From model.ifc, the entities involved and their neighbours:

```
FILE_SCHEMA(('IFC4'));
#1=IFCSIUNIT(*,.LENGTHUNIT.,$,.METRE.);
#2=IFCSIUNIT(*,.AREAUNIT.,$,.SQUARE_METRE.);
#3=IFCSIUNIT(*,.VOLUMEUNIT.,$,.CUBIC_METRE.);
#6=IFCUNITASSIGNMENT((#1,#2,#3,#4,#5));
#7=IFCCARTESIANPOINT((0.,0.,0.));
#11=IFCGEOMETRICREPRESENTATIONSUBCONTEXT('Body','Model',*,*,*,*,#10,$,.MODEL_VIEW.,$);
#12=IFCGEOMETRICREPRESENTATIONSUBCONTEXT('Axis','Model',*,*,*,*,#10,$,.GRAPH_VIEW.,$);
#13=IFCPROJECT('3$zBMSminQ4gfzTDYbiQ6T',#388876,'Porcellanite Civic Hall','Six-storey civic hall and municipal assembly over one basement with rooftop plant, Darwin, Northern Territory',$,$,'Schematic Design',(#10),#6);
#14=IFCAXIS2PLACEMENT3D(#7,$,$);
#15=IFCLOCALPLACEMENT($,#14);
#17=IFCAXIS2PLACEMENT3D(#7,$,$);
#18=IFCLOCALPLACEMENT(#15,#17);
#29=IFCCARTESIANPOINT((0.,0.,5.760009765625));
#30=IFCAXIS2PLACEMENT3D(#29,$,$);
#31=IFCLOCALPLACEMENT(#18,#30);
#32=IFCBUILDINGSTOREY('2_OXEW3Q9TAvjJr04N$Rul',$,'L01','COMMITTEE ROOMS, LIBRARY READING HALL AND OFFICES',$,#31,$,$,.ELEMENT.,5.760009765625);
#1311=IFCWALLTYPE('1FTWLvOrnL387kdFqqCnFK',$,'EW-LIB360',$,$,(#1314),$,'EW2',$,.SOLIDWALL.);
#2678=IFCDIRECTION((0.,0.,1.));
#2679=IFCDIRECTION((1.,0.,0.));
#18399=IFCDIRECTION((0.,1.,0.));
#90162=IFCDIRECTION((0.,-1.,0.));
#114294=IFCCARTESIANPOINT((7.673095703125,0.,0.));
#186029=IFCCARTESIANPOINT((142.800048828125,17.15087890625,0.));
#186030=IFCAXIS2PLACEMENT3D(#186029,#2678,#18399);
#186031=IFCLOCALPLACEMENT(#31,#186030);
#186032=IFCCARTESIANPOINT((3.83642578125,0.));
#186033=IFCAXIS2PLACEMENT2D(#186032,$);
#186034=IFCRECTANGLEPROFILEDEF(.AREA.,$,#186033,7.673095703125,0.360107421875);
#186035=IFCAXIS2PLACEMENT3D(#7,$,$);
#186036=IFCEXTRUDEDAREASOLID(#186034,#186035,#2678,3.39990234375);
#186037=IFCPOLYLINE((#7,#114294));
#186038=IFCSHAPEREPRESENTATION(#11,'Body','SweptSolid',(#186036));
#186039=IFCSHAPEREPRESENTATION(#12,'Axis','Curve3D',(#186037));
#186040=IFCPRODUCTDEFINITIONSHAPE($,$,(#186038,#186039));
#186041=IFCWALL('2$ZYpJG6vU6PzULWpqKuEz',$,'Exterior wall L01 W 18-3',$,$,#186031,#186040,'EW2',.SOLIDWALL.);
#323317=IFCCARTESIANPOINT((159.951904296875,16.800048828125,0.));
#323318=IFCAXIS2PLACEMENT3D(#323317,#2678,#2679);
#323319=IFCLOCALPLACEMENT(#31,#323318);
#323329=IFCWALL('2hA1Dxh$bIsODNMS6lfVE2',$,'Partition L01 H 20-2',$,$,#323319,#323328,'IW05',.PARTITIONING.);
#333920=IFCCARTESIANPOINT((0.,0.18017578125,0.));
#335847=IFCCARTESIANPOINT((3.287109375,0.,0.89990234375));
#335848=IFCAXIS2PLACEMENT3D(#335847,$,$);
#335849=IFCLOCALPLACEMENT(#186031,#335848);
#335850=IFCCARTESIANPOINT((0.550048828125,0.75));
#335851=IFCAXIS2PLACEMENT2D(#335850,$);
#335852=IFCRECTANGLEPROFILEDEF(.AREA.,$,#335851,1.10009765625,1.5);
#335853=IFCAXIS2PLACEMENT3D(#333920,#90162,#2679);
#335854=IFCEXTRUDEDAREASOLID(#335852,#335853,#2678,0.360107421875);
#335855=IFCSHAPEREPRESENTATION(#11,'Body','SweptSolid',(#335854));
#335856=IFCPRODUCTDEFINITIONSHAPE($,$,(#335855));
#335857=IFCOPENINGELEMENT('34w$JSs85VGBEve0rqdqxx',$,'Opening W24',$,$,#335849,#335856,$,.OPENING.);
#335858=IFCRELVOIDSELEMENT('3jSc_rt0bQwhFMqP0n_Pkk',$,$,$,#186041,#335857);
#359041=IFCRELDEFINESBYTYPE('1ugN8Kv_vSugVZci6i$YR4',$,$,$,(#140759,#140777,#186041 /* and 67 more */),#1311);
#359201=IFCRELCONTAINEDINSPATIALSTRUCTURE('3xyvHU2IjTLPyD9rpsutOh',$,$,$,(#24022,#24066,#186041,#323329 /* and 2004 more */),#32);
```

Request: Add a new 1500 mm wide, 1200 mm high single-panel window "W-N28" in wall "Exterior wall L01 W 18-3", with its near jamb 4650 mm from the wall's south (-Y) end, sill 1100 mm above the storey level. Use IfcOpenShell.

```python
import numpy as np
import ifcopenshell
import ifcopenshell.api.feature
import ifcopenshell.api.geometry
import ifcopenshell.api.root
import ifcopenshell.api.spatial
import ifcopenshell.geom
import ifcopenshell.util.element
import ifcopenshell.util.placement
import ifcopenshell.util.representation
import ifcopenshell.util.shape
import ifcopenshell.util.unit

model = ifcopenshell.open("model.ifc")
unit_scale = ifcopenshell.util.unit.calculate_unit_scale(model)
settings = ifcopenshell.geom.settings()


def volume(element):
    """Net volume in cubic metres, openings subtracted."""
    shape = ifcopenshell.geom.create_shape(settings, element)
    return ifcopenshell.util.shape.get_volume(shape.geometry)


wall = model.by_guid("2$ZYpJG6vU6PzULWpqKuEz")
storey = ifcopenshell.util.element.get_container(wall, ifc_class="IfcBuildingStorey")
context = ifcopenshell.util.representation.get_context(model, "Model", "Body", "MODEL_VIEW")
before = volume(wall)

width, height, from_end, sill = 1.5, 1.2, 4.65, 1.1  # metres

# The wall runs along its own X axis, and the end named is its -X end.
wall_shape = ifcopenshell.geom.create_shape(settings, wall)
x, y, z = ifcopenshell.util.shape.get_vertices(wall_shape.geometry).T
start = x.min() + from_end
face, thickness = float(y.min()), float(y.max() - y.min())
wall_matrix = ifcopenshell.util.placement.get_local_placement(wall.ObjectPlacement)
level = ifcopenshell.util.placement.get_local_placement(storey.ObjectPlacement)[2, 3]


def in_wall(x, y):
    """Placement at x, y metres in the wall's axes, at sill height."""
    matrix = wall_matrix.copy()
    matrix[:, 3] = wall_matrix @ np.array([x / unit_scale, y / unit_scale, 0.0, 1.0])
    matrix[2, 3] = level + sill / unit_scale
    return matrix


# Opening: a box that overshoots both wall faces by 50 mm.
opening = ifcopenshell.api.root.create_entity(model, ifc_class="IfcOpeningElement", predefined_type="OPENING")
box = ifcopenshell.api.geometry.add_wall_representation(
    model, context=context, length=width, height=height, thickness=thickness + 0.1
)
ifcopenshell.api.geometry.assign_representation(model, product=opening, representation=box)
ifcopenshell.api.geometry.edit_object_placement(model, product=opening, matrix=in_wall(start, face - 0.05), is_si=False)
ifcopenshell.api.feature.add_feature(model, feature=opening, element=wall)

window = ifcopenshell.api.root.create_entity(model, ifc_class="IfcWindow", name="W-N28", predefined_type="WINDOW")
window.OverallWidth, window.OverallHeight = width / unit_scale, height / unit_scale
window.PartitioningType = "SINGLE_PANEL"
body = ifcopenshell.api.geometry.add_window_representation(
    model,
    context=context,
    overall_width=window.OverallWidth,
    overall_height=window.OverallHeight,
    partition_type="SINGLE_PANEL",
)
ifcopenshell.api.geometry.assign_representation(model, product=window, representation=body)
ifcopenshell.api.spatial.assign_container(model, products=[window], relating_structure=storey)
ifcopenshell.api.feature.add_filling(model, opening=opening, element=window)

# Centre the window in the wall's thickness.
ifcopenshell.api.geometry.edit_object_placement(model, product=window, matrix=in_wall(start, face), is_si=False)
window_shape = ifcopenshell.geom.create_shape(settings, window)
depth = ifcopenshell.util.shape.get_vertices(window_shape.geometry)[:, 1]
offset = face + thickness / 2 - (depth.min() + depth.max()) / 2
ifcopenshell.api.geometry.edit_object_placement(model, product=window, matrix=in_wall(start, offset), is_si=False)

after = volume(wall)

print(f"wall volume {before:.3f} -> {after:.3f} m3")

model.write("model-out.ifc")
```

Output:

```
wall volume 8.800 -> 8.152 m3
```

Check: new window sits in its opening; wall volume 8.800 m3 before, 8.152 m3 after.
